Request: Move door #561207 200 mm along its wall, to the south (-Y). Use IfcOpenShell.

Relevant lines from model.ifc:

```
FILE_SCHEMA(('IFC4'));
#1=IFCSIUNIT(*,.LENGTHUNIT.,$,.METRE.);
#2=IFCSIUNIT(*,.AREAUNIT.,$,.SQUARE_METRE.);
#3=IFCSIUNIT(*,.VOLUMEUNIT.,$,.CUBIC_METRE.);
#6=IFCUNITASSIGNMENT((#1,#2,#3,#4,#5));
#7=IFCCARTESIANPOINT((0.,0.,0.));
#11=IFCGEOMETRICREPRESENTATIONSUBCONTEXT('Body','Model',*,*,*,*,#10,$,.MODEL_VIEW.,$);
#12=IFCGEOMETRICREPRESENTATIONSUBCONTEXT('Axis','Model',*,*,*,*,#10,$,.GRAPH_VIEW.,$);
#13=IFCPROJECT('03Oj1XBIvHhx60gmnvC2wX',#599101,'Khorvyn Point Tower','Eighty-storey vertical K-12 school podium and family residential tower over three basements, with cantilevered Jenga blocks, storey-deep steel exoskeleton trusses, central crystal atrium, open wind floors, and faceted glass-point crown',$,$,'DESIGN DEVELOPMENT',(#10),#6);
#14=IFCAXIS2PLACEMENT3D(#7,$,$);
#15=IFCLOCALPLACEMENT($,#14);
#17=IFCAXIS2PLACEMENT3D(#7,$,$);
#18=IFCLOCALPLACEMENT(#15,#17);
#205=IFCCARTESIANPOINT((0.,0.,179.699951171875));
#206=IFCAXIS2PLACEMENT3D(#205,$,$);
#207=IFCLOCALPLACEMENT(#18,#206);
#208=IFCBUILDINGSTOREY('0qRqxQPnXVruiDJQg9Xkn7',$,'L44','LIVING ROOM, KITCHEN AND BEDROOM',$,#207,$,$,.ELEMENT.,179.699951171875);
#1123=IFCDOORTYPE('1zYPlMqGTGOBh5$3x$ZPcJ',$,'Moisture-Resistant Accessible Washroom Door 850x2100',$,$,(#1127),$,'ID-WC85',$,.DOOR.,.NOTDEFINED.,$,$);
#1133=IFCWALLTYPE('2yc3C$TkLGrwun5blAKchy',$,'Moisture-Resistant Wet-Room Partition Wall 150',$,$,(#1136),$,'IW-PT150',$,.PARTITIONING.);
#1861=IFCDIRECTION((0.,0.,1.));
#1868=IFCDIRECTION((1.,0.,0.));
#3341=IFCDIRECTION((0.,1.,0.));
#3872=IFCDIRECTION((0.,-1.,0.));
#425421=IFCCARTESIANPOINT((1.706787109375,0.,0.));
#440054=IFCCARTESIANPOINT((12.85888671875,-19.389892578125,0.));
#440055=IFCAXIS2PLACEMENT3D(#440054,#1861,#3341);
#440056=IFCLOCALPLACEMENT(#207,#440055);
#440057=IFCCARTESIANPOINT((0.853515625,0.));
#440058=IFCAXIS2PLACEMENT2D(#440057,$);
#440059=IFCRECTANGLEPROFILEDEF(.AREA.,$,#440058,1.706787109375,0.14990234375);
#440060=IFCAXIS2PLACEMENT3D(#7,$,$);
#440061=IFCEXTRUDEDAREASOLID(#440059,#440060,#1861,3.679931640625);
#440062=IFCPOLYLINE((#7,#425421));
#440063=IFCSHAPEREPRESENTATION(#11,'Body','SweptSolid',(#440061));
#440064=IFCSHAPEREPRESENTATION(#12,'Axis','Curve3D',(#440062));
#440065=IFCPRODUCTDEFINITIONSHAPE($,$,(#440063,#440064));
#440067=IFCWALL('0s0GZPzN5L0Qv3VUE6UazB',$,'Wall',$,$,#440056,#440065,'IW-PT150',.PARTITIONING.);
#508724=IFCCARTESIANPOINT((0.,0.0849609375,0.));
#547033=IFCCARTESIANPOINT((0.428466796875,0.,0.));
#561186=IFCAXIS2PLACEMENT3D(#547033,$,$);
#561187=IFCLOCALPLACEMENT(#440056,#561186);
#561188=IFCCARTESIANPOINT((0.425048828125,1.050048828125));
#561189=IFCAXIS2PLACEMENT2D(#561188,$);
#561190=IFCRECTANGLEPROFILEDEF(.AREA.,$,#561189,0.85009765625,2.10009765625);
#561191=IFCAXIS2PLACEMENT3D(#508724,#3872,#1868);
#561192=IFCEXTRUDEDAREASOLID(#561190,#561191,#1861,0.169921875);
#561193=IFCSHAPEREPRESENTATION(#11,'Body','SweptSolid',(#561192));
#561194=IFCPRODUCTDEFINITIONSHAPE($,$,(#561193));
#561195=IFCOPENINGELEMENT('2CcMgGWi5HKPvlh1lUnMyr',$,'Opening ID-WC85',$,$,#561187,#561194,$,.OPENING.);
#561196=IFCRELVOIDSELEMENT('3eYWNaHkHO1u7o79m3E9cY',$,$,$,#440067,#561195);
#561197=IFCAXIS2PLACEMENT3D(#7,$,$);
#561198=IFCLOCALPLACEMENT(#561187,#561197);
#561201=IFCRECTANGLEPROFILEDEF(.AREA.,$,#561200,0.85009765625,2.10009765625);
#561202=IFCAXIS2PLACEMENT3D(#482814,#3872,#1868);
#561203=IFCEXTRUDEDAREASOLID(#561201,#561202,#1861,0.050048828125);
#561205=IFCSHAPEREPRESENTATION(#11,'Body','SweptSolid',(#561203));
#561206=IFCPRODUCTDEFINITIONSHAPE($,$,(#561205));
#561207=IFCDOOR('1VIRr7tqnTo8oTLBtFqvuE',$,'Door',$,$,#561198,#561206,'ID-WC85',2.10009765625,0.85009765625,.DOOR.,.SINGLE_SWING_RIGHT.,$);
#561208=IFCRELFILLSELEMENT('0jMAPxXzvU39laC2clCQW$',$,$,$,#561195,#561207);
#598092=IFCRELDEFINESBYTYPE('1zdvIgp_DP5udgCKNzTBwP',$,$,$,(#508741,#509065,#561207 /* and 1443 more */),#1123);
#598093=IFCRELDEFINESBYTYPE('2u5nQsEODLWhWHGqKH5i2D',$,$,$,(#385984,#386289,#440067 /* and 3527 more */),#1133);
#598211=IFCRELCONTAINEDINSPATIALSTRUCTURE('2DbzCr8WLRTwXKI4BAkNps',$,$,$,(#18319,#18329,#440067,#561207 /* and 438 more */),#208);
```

```python
import ifcopenshell
import ifcopenshell.api.geometry
import ifcopenshell.util.placement

model = ifcopenshell.open("model.ifc")

door = model.by_id(561207)
opening = door.FillsVoids[0].RelatingOpeningElement
wall = opening.VoidsElements[0].RelatingBuildingElement

wall_matrix = ifcopenshell.util.placement.get_local_placement(wall.ObjectPlacement)
shift = wall_matrix[:3, 0] * -0.2
before = ifcopenshell.util.placement.get_local_placement(door.ObjectPlacement)[:3, 3].copy()

# The door is placed relative to its opening, so it follows when the opening moves.
matrix = ifcopenshell.util.placement.get_local_placement(opening.ObjectPlacement)
matrix[:3, 3] += shift
ifcopenshell.api.geometry.edit_object_placement(
    model, product=opening, matrix=matrix, is_si=False, should_transform_children=True
)

after = ifcopenshell.util.placement.get_local_placement(door.ObjectPlacement)[:3, 3]
print("door moved by", (after - before).round(3) + 0.0)

model.write("model_v2.ifc")
```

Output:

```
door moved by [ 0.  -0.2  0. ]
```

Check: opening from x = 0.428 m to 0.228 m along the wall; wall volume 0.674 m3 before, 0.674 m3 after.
